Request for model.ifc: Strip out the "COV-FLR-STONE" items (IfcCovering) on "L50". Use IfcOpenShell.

First a look at what the model holds.

```python
import ifcopenshell
import ifcopenshell.util.element

model = ifcopenshell.open("model.ifc")
print(model.schema)
storey = next(s for s in model.by_type("IfcBuildingStorey") if s.Name == "L50")
coverings = [e for e in ifcopenshell.util.element.get_decomposition(storey) if e.is_a("IfcCovering")]
seen = {}
for e in coverings:
    element_type = ifcopenshell.util.element.get_type(e)
    name = element_type.Name if element_type not in (None, e) else None
    seen[name] = seen.get(name, 0) + 1
for name, count in sorted(seen.items(), key=str):
    print(count, "x", name)
```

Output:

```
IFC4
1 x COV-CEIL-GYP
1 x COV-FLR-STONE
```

```python
import ifcopenshell
import ifcopenshell.api.root
import ifcopenshell.util.element

model = ifcopenshell.open("model.ifc")

storey = next(s for s in model.by_type("IfcBuildingStorey") if s.Name == "L50")
coverings = [e for e in ifcopenshell.util.element.get_decomposition(storey) if e.is_a("IfcCovering")]
targets = [e for e in coverings if (t := ifcopenshell.util.element.get_type(e)) not in (None, e) and t.Name == "COV-FLR-STONE"]

for e in targets:
    ifcopenshell.api.root.remove_product(model, product=e)
print(len(targets), "removed")

model.write("model_updated.ifc")
```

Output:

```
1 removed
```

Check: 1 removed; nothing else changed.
